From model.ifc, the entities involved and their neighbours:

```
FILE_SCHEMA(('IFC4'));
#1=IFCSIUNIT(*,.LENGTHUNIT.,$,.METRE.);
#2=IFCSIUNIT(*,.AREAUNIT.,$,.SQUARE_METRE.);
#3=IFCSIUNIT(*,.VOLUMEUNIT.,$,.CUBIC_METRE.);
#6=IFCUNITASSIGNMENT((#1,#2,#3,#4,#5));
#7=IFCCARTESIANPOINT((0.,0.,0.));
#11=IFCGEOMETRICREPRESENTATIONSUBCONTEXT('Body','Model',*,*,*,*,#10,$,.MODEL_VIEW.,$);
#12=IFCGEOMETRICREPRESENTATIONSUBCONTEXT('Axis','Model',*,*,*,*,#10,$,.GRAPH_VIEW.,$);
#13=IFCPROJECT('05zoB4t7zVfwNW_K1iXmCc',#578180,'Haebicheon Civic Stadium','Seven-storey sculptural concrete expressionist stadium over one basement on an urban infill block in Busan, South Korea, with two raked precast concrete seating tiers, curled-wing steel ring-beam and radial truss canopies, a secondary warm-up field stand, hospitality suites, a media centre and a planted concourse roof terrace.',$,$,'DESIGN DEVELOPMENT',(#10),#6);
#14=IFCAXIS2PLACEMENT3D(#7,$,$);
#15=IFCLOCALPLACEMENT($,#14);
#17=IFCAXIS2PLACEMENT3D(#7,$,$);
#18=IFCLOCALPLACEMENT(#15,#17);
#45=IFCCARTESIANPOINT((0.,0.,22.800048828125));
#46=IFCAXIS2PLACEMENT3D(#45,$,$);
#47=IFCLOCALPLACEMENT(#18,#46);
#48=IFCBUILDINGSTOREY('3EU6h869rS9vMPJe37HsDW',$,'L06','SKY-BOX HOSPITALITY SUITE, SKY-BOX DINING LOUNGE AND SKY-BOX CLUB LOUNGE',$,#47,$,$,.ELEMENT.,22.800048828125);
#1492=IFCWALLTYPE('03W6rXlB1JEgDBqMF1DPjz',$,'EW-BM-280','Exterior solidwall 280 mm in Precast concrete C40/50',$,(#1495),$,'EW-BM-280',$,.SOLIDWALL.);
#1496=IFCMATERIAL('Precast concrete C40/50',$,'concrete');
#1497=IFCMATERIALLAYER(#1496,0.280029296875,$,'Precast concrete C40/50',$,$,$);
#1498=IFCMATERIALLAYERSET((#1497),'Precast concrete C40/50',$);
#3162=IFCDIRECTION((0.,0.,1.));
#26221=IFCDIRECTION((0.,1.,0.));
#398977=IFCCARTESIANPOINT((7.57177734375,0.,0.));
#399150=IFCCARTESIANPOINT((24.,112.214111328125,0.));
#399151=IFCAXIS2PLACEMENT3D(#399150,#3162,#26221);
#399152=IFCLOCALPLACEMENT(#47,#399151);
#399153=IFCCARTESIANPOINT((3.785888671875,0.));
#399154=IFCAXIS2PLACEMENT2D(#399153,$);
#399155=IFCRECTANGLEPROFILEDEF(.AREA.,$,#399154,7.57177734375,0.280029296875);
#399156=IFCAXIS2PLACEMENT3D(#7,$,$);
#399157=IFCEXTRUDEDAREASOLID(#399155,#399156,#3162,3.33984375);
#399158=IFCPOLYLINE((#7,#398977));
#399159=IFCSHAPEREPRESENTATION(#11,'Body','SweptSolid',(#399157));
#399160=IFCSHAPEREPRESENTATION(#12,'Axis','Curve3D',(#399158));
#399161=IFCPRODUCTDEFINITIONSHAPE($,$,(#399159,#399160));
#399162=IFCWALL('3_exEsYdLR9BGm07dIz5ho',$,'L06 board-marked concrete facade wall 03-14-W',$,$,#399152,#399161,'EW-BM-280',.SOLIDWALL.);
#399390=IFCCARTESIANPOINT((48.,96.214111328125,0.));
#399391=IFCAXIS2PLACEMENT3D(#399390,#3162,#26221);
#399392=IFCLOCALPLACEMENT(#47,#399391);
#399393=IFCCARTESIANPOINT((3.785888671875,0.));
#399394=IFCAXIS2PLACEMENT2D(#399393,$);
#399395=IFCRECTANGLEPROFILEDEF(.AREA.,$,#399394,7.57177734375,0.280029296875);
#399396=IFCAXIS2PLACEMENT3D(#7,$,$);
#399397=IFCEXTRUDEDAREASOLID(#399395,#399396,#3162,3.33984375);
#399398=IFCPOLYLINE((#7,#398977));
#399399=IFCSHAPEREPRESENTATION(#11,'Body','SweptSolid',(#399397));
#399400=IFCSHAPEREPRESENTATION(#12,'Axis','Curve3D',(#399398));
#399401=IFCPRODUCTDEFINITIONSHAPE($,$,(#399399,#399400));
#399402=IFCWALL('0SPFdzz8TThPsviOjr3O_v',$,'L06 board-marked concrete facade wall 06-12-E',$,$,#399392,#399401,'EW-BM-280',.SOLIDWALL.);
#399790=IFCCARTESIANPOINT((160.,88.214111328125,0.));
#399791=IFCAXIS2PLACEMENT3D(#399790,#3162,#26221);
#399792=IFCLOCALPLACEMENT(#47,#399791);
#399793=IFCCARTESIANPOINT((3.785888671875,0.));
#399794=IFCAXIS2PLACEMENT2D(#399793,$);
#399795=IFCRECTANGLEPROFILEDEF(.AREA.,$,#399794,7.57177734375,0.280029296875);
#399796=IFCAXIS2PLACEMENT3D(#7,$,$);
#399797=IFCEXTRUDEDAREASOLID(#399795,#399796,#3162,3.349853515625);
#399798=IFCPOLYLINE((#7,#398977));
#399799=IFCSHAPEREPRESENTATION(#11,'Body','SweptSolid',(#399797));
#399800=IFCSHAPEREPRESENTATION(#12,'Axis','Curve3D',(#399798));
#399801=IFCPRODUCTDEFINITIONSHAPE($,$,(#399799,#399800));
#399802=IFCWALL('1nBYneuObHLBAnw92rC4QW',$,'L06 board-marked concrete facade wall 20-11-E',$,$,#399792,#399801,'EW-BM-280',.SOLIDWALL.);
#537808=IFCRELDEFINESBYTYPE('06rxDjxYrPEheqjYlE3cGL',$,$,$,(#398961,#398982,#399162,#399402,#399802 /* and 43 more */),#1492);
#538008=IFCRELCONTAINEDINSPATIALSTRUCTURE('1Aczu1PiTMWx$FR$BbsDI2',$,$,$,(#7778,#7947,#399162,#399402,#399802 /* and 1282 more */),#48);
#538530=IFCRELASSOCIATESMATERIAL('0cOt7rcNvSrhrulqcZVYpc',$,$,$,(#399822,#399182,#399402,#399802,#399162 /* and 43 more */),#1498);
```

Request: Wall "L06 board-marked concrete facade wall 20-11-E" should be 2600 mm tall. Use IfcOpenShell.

```python
import ifcopenshell
import ifcopenshell.geom
import ifcopenshell.util.representation
import ifcopenshell.util.shape
import ifcopenshell.util.unit

model = ifcopenshell.open("model.ifc")
unit_scale = ifcopenshell.util.unit.calculate_unit_scale(model)
settings = ifcopenshell.geom.settings()


def volume(element):
    """Net volume in cubic metres, openings subtracted."""
    shape = ifcopenshell.geom.create_shape(settings, element)
    return ifcopenshell.util.shape.get_volume(shape.geometry)


wall = model.by_guid("1nBYneuObHLBAnw92rC4QW")
before = volume(wall)

body = ifcopenshell.util.representation.get_representation(wall, "Model", "Body")
solid = body.Items[0]
old_height = solid.Depth
solid.Depth = 2.6 / unit_scale
after = volume(wall)

print(f"height {old_height:g} -> {solid.Depth:g}, volume {before:.3f} -> {after:.3f} m3")

model.write("model-out.ifc")
```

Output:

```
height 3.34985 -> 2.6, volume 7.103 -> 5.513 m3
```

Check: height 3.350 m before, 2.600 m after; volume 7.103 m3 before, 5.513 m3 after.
